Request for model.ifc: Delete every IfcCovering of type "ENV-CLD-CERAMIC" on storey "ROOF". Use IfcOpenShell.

First a look at what the model holds.

```python
import ifcopenshell
import ifcopenshell.util.element

model = ifcopenshell.open("model.ifc")
print(model.schema)
storey = next(s for s in model.by_type("IfcBuildingStorey") if s.Name == "ROOF")
coverings = [e for e in ifcopenshell.util.element.get_decomposition(storey) if e.is_a("IfcCovering")]
seen = {}
for e in coverings:
    element_type = ifcopenshell.util.element.get_type(e)
    name = element_type.Name if element_type not in (None, e) else None
    seen[name] = seen.get(name, 0) + 1
for name, count in sorted(seen.items(), key=str):
    print(count, "x", name)
```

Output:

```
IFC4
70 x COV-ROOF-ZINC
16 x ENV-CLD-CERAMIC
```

```python
import ifcopenshell
import ifcopenshell.api.root
import ifcopenshell.util.element

model = ifcopenshell.open("model.ifc")

storey = next(s for s in model.by_type("IfcBuildingStorey") if s.Name == "ROOF")
coverings = [e for e in ifcopenshell.util.element.get_decomposition(storey) if e.is_a("IfcCovering")]
targets = [e for e in coverings if (t := ifcopenshell.util.element.get_type(e)) not in (None, e) and t.Name == "ENV-CLD-CERAMIC"]

for e in targets:
    ifcopenshell.api.root.remove_product(model, product=e)
print(len(targets), "removed")

model.write("model_rev.ifc")
```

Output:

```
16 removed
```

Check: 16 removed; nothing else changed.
